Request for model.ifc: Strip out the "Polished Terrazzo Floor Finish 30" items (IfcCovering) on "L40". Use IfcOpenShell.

First a look at what the model holds.

```python
import ifcopenshell
import ifcopenshell.util.element

model = ifcopenshell.open("model.ifc")
print(model.schema)
storey = next(s for s in model.by_type("IfcBuildingStorey") if s.Name == "L40")
coverings = [e for e in ifcopenshell.util.element.get_decomposition(storey) if e.is_a("IfcCovering")]
seen = {}
for e in coverings:
    element_type = ifcopenshell.util.element.get_type(e)
    name = element_type.Name if element_type not in (None, e) else None
    seen[name] = seen.get(name, 0) + 1
for name, count in sorted(seen.items(), key=str):
    print(count, "x", name)
```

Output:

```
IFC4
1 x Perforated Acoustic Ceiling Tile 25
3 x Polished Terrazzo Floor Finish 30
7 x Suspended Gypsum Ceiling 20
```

```python
import ifcopenshell
import ifcopenshell.api.root
import ifcopenshell.util.element

model = ifcopenshell.open("model.ifc")

storey = next(s for s in model.by_type("IfcBuildingStorey") if s.Name == "L40")
coverings = [e for e in ifcopenshell.util.element.get_decomposition(storey) if e.is_a("IfcCovering")]
targets = [e for e in coverings if (t := ifcopenshell.util.element.get_type(e)) not in (None, e) and t.Name == "Polished Terrazzo Floor Finish 30"]

for e in targets:
    ifcopenshell.api.root.remove_product(model, product=e)
print(len(targets), "removed")

model.write("model-out.ifc")
```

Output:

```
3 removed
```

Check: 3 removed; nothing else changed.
